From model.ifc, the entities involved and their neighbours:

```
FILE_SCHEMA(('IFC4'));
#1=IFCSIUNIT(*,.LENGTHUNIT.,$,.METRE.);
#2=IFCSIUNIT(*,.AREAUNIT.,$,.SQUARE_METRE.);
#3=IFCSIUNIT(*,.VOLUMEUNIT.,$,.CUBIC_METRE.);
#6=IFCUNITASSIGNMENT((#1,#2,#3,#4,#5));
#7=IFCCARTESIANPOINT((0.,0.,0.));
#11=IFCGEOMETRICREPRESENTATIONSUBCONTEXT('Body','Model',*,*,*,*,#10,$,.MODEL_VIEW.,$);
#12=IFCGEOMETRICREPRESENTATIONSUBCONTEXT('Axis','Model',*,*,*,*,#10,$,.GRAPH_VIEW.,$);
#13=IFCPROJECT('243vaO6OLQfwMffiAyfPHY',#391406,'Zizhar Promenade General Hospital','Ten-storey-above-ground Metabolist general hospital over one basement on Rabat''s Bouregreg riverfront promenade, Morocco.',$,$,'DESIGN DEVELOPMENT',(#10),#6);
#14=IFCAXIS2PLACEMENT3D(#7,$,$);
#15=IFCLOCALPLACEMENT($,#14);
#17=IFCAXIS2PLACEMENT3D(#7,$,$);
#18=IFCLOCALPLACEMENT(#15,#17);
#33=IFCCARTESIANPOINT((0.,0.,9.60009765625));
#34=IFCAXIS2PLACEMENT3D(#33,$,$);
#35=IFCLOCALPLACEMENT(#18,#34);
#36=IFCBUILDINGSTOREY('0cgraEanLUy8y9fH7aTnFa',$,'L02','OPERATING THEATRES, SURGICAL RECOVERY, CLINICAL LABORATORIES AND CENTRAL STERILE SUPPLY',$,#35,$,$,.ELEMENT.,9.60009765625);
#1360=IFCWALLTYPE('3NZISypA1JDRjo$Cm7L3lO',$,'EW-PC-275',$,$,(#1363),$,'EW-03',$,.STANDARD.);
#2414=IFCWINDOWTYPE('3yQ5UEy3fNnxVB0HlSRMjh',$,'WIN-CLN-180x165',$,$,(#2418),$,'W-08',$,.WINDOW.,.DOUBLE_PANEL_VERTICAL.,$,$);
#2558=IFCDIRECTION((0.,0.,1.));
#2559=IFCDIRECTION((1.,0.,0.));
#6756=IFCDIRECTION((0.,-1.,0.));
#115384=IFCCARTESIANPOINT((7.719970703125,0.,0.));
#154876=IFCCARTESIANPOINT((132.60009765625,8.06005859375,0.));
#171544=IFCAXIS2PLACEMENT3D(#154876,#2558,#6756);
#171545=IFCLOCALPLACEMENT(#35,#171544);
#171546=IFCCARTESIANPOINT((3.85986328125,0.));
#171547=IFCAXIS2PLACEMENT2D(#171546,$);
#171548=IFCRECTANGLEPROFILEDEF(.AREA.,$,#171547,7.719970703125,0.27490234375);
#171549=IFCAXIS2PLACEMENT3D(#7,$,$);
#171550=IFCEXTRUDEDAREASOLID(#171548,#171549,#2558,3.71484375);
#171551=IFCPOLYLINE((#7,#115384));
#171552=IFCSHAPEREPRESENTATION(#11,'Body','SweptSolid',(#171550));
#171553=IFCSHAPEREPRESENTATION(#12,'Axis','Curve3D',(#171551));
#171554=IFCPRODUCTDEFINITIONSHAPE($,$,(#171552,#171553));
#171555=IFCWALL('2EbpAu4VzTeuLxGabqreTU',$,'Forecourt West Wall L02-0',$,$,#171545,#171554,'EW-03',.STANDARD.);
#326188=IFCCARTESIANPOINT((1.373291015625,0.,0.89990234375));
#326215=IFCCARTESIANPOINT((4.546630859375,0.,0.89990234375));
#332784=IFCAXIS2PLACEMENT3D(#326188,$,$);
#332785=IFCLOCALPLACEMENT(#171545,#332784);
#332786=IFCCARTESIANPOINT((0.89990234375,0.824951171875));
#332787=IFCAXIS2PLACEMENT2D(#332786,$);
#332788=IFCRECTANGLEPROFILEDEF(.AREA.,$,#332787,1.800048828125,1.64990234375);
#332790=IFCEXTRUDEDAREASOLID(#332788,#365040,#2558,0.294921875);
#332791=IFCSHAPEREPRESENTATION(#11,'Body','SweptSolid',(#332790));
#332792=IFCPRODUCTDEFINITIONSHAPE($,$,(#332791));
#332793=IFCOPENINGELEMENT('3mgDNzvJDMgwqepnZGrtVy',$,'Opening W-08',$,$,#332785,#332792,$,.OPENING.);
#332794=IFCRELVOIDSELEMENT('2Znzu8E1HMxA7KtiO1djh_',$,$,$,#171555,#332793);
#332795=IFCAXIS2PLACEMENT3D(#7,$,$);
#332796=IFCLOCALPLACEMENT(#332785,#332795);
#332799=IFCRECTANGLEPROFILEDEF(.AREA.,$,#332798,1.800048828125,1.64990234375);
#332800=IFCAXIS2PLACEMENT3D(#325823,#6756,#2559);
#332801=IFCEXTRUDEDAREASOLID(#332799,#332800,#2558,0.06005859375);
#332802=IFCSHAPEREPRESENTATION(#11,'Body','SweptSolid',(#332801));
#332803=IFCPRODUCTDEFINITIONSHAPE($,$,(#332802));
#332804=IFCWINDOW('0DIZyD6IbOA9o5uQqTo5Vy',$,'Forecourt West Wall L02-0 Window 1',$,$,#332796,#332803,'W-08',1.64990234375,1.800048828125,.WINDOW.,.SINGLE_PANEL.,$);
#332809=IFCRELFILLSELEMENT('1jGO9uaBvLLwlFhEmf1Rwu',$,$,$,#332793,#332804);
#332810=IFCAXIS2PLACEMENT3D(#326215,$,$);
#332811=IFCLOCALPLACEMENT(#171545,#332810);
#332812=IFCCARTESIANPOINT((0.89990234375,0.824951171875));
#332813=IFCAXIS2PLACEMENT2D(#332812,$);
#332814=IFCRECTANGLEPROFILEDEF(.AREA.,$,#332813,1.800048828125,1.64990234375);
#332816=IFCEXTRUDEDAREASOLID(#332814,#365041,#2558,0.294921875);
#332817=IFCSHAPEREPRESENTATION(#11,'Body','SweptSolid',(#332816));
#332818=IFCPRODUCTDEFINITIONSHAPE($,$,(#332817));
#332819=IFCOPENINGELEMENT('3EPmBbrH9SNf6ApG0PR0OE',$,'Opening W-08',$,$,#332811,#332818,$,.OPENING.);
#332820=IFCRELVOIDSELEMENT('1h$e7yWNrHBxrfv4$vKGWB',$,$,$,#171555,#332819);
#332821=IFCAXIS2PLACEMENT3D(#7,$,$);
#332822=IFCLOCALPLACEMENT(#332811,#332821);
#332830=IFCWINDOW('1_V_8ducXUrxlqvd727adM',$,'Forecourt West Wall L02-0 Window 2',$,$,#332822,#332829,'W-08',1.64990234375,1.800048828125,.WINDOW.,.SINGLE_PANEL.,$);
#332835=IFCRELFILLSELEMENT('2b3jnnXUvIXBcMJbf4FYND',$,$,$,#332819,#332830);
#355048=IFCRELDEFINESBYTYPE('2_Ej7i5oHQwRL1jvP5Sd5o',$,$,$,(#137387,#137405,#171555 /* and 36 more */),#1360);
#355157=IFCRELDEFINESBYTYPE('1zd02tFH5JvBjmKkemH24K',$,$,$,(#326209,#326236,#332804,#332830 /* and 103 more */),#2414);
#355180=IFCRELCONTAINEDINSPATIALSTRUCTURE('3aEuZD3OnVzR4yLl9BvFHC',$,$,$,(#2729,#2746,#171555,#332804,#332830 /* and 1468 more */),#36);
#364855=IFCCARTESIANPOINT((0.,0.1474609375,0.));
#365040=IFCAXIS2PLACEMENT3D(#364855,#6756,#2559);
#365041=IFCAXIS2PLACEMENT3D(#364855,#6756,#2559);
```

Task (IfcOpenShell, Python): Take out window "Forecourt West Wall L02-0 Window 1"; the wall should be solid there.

```python
import ifcopenshell
import ifcopenshell.api.feature
import ifcopenshell.api.root
import ifcopenshell.geom
import ifcopenshell.util.shape

model = ifcopenshell.open("model.ifc")
settings = ifcopenshell.geom.settings()


def volume(element):
    """Net volume in cubic metres, openings subtracted."""
    shape = ifcopenshell.geom.create_shape(settings, element)
    return ifcopenshell.util.shape.get_volume(shape.geometry)


window = model.by_id(332804)
opening = window.FillsVoids[0].RelatingOpeningElement
wall = opening.VoidsElements[0].RelatingBuildingElement
before = volume(wall)

ifcopenshell.api.root.remove_product(model, product=window)
ifcopenshell.api.feature.remove_feature(model, feature=opening)

after = volume(wall)

print(f"wall volume {before:.3f} -> {after:.3f} m3")

model.write("model-out.ifc")
```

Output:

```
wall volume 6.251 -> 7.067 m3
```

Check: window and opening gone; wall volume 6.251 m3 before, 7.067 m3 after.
